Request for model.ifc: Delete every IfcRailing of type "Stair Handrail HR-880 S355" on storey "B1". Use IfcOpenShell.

First a look at what the model holds.

```python
import ifcopenshell
import ifcopenshell.util.element

model = ifcopenshell.open("model.ifc")
print(model.schema)
storey = next(s for s in model.by_type("IfcBuildingStorey") if s.Name == "B1")
railings = [e for e in ifcopenshell.util.element.get_decomposition(storey) if e.is_a("IfcRailing")]
seen = {}
for e in railings:
    element_type = ifcopenshell.util.element.get_type(e)
    name = element_type.Name if element_type not in (None, e) else None
    seen[name] = seen.get(name, 0) + 1
for name, count in sorted(seen.items(), key=str):
    print(count, "x", name)
```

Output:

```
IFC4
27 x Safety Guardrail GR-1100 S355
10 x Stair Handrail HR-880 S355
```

```python
import ifcopenshell
import ifcopenshell.api.root
import ifcopenshell.util.element

model = ifcopenshell.open("model.ifc")

storey = next(s for s in model.by_type("IfcBuildingStorey") if s.Name == "B1")
railings = [e for e in ifcopenshell.util.element.get_decomposition(storey) if e.is_a("IfcRailing")]
targets = [e for e in railings if (t := ifcopenshell.util.element.get_type(e)) not in (None, e) and t.Name == "Stair Handrail HR-880 S355"]

for e in targets:
    ifcopenshell.api.root.remove_product(model, product=e)
print(len(targets), "removed")

model.write("model-out.ifc")
```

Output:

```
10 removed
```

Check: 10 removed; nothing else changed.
